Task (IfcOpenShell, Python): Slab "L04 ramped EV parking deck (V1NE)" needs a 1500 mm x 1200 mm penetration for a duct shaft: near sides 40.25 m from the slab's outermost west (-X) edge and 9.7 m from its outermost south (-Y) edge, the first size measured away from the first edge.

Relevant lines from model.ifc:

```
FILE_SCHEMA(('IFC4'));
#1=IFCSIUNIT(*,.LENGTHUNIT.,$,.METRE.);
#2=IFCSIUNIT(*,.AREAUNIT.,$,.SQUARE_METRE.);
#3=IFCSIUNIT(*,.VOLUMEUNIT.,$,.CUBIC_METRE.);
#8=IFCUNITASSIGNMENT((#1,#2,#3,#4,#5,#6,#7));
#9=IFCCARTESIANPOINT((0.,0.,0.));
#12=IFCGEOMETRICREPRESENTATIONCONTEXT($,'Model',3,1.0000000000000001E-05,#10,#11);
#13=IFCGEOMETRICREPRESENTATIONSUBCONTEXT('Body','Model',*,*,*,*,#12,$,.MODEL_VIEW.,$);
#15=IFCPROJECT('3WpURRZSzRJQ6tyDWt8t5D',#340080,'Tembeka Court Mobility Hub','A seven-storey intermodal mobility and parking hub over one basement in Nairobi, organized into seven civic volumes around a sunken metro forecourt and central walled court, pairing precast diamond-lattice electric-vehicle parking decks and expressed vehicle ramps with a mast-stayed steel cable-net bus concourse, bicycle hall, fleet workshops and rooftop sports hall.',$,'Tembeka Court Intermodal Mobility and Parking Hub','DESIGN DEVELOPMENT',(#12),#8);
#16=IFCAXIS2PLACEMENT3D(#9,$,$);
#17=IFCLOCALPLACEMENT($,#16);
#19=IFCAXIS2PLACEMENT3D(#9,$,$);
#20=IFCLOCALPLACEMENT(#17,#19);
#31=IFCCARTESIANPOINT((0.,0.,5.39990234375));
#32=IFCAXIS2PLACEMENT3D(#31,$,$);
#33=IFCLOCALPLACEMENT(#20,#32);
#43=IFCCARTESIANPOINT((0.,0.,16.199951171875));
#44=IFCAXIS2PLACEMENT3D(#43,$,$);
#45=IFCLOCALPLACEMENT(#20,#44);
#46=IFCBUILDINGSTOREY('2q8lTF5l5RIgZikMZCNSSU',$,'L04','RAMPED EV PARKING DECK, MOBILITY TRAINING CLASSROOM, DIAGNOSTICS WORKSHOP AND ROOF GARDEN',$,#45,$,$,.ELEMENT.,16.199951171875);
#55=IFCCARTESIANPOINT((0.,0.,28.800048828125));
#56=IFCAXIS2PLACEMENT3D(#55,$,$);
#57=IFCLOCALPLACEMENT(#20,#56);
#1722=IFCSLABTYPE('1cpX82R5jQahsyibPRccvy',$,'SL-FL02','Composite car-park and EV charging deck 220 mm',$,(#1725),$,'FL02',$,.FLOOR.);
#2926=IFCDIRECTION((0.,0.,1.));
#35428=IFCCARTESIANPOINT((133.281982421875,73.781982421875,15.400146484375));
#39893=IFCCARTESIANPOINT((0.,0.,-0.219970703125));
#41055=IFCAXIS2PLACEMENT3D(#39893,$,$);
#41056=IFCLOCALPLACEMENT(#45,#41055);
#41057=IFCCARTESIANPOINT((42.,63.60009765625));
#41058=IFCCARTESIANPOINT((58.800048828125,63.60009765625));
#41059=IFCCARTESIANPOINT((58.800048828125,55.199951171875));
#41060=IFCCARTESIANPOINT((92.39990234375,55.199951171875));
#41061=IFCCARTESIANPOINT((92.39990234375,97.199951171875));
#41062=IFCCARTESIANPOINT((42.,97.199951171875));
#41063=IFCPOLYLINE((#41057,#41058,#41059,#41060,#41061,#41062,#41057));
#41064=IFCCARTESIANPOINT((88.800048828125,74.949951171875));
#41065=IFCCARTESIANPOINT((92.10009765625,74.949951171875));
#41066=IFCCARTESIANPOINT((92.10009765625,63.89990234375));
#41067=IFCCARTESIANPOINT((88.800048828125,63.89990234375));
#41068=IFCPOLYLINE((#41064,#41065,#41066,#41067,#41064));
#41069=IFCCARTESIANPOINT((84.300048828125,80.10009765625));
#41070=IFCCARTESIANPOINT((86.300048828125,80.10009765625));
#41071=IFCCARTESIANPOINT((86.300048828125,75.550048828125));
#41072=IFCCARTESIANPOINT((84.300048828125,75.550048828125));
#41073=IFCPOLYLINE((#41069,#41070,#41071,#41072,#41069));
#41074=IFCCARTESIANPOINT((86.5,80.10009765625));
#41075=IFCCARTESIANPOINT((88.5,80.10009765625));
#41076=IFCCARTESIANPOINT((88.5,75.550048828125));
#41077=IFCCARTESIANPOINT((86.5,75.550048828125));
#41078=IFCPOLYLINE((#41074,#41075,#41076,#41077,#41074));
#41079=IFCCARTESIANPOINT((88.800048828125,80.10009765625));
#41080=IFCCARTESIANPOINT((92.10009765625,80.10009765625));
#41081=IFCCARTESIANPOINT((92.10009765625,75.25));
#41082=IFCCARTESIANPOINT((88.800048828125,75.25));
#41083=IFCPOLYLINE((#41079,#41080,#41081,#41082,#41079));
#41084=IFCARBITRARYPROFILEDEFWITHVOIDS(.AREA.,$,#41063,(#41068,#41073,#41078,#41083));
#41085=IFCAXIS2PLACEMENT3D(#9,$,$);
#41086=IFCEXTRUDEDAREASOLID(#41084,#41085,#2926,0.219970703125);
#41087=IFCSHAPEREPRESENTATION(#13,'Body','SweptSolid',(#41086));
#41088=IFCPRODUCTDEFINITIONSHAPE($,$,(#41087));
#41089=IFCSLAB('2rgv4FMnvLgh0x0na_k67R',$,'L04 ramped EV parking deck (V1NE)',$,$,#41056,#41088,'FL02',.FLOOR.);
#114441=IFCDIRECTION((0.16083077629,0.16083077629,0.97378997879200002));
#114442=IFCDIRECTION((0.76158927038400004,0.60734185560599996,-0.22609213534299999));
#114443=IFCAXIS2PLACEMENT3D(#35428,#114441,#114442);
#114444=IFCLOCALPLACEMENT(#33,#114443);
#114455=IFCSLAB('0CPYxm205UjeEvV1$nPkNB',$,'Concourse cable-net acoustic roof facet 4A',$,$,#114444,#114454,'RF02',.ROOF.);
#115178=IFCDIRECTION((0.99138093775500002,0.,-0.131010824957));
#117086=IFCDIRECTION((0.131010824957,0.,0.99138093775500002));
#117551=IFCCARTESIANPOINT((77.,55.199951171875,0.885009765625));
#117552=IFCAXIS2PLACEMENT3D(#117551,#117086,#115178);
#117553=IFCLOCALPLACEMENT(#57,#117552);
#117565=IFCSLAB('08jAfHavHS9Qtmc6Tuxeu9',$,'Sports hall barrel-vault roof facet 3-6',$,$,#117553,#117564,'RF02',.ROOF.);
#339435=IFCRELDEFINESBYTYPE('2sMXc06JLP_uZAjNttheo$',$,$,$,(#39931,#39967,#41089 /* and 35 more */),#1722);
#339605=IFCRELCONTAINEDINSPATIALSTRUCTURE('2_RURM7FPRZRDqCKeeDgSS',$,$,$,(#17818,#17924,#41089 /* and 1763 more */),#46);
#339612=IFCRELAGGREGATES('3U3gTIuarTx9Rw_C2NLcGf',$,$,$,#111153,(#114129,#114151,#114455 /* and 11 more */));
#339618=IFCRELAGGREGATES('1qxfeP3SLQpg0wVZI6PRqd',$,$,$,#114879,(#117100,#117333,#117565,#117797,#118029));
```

```python
import numpy as np
import ifcopenshell
import ifcopenshell.api.feature
import ifcopenshell.api.geometry
import ifcopenshell.api.root
import ifcopenshell.geom
import ifcopenshell.util.placement
import ifcopenshell.util.representation
import ifcopenshell.util.shape
import ifcopenshell.util.unit

model = ifcopenshell.open("model.ifc")
unit_scale = ifcopenshell.util.unit.calculate_unit_scale(model)
settings = ifcopenshell.geom.settings()


def volume(element):
    """Net volume in cubic metres, openings subtracted."""
    shape = ifcopenshell.geom.create_shape(settings, element)
    return ifcopenshell.util.shape.get_volume(shape.geometry)


slab = model.by_guid("2rgv4FMnvLgh0x0na_k67R")
before = volume(slab)

# Extent in the slab's own axes, in metres. The edges named are its -X and -Y sides.
slab_shape = ifcopenshell.geom.create_shape(settings, slab)
vertices = ifcopenshell.util.shape.get_vertices(slab_shape.geometry)
x_min, y_min, bottom = vertices.min(axis=0)
top = vertices[:, 2].max()

opening = ifcopenshell.api.root.create_entity(model, ifc_class="IfcOpeningElement", name="Duct shaft opening", predefined_type="OPENING")
context = ifcopenshell.util.representation.get_context(model, "Model", "Body", "MODEL_VIEW")
width, depth = 1.5, 1.2
outline = [(0.0, 0.0), (width, 0.0), (width, depth), (0.0, depth), (0.0, 0.0)]
# Overshoot both faces by 50 mm so the cut is clean.
shape = ifcopenshell.api.geometry.add_slab_representation(
    model, context=context, depth=top - bottom + 0.1, polyline=outline
)
ifcopenshell.api.geometry.assign_representation(model, product=opening, representation=shape)

matrix = ifcopenshell.util.placement.get_local_placement(slab.ObjectPlacement)
matrix[:, 3] = matrix @ np.append(np.array([x_min + 40.25, y_min + 9.7, bottom - 0.05]) / unit_scale, 1.0)
ifcopenshell.api.geometry.edit_object_placement(model, product=opening, matrix=matrix, is_si=False)
ifcopenshell.api.feature.add_feature(model, feature=opening, element=slab)

after = volume(slab)

print(f"slab volume {before:.3f} -> {after:.3f} m3")

model.write("model-out.ifc")
```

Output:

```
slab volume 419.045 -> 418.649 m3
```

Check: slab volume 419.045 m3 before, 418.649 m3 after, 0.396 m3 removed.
